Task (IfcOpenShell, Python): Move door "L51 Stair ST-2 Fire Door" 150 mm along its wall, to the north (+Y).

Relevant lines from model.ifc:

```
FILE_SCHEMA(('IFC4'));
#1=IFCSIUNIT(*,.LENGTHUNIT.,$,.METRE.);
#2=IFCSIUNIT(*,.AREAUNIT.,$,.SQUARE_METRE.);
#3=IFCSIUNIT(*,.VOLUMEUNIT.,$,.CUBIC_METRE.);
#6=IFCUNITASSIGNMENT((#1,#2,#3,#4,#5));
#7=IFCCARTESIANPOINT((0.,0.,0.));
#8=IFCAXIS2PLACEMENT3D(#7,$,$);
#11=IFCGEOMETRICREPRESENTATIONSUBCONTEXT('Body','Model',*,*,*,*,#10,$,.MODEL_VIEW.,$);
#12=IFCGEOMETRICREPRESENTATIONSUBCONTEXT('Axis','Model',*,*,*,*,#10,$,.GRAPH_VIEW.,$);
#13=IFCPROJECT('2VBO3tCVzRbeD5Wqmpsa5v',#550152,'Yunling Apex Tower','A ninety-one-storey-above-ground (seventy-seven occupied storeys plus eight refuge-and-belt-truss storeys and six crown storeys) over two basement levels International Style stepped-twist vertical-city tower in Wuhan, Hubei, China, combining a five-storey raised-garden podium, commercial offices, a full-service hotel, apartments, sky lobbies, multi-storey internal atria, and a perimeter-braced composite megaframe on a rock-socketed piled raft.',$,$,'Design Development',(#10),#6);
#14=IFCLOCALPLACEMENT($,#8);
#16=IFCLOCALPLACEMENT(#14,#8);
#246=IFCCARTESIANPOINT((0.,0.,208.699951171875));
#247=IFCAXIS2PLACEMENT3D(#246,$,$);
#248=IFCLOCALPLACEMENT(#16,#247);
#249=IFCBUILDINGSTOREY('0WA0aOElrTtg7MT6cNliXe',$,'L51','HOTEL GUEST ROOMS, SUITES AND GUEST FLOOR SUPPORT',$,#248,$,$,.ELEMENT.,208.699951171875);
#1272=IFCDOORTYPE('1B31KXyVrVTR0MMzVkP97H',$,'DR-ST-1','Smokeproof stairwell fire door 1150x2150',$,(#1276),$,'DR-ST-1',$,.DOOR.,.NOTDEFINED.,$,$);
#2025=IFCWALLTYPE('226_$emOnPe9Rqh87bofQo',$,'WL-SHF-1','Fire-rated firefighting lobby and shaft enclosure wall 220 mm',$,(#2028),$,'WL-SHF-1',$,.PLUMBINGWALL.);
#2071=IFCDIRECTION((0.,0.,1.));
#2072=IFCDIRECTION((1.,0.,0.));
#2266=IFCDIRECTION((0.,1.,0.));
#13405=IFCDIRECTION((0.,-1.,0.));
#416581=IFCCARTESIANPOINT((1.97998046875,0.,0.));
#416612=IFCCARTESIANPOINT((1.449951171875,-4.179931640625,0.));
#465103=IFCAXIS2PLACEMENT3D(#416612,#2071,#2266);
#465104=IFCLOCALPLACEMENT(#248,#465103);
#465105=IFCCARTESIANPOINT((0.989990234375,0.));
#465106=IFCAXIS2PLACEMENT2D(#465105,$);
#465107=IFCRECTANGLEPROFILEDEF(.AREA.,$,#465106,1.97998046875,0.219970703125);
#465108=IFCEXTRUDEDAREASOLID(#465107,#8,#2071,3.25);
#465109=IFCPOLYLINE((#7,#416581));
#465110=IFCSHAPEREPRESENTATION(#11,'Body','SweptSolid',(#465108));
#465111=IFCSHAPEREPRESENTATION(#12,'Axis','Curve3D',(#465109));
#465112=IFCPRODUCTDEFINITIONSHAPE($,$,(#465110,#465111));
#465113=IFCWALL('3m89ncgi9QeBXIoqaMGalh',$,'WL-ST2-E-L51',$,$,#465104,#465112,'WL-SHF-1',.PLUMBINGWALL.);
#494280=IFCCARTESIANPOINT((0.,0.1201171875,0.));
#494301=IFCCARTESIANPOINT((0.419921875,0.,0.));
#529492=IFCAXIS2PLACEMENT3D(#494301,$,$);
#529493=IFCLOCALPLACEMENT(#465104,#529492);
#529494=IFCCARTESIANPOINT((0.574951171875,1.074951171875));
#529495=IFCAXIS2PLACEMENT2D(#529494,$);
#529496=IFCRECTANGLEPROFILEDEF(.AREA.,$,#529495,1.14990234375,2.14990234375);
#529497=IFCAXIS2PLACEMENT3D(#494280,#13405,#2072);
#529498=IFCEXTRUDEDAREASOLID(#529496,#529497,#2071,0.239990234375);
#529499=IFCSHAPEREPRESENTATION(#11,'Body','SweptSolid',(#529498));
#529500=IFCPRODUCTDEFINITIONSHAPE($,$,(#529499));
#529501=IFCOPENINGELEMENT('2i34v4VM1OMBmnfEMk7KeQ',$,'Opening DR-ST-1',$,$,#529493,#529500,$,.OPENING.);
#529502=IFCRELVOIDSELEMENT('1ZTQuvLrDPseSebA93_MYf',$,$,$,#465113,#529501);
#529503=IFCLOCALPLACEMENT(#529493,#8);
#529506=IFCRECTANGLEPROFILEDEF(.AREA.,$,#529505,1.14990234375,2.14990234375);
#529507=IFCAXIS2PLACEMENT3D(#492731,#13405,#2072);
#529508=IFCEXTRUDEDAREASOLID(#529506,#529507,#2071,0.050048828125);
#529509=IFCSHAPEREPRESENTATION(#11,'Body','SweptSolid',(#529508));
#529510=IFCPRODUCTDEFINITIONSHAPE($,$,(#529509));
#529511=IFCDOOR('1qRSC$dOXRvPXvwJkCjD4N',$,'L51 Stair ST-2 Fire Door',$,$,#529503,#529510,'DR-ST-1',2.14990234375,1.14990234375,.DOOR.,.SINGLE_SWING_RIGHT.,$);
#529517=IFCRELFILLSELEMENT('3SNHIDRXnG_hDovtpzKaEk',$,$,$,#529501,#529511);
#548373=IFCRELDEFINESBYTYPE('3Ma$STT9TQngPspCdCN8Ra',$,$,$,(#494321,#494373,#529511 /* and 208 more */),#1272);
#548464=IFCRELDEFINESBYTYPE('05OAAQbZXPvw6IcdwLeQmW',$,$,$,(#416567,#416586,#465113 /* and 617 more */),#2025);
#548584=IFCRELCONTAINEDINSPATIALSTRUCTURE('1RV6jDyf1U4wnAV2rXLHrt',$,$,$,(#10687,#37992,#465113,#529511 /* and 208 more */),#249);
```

```python
import ifcopenshell
import ifcopenshell.api.geometry
import ifcopenshell.util.placement

model = ifcopenshell.open("model.ifc")

door = model.by_guid("1qRSC$dOXRvPXvwJkCjD4N")
opening = door.FillsVoids[0].RelatingOpeningElement
wall = opening.VoidsElements[0].RelatingBuildingElement

wall_matrix = ifcopenshell.util.placement.get_local_placement(wall.ObjectPlacement)
shift = wall_matrix[:3, 0] * 0.15
before = ifcopenshell.util.placement.get_local_placement(door.ObjectPlacement)[:3, 3].copy()

# The door is placed relative to its opening, so it follows when the opening moves.
matrix = ifcopenshell.util.placement.get_local_placement(opening.ObjectPlacement)
matrix[:3, 3] += shift
ifcopenshell.api.geometry.edit_object_placement(
    model, product=opening, matrix=matrix, is_si=False, should_transform_children=True
)

after = ifcopenshell.util.placement.get_local_placement(door.ObjectPlacement)[:3, 3]
print("door moved by", (after - before).round(3) + 0.0)

model.write("model_updated.ifc")
```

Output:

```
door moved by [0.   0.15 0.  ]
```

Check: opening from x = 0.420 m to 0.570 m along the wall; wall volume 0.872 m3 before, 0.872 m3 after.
